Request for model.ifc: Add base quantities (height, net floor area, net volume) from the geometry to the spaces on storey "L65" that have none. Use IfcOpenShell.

First a look at what the model holds.

```python
import ifcopenshell
import ifcopenshell.util.element
import ifcopenshell.util.unit

model = ifcopenshell.open("model.ifc")
print(model.schema)
for unit_type in ("LENGTHUNIT", "AREAUNIT", "VOLUMEUNIT"):
    print(unit_type, ifcopenshell.util.unit.calculate_unit_scale(model, unit_type))
storey = next(s for s in model.by_type("IfcBuildingStorey") if s.Name == "L65")
spaces = [e for e in ifcopenshell.util.element.get_decomposition(storey) if e.is_a("IfcSpace")]
for e in sorted(spaces, key=lambda e: e.id()):
    print(e.id(), e.is_a(), e.Name, list(ifcopenshell.util.element.get_psets(e, qtos_only=True)), sep=" | ")
```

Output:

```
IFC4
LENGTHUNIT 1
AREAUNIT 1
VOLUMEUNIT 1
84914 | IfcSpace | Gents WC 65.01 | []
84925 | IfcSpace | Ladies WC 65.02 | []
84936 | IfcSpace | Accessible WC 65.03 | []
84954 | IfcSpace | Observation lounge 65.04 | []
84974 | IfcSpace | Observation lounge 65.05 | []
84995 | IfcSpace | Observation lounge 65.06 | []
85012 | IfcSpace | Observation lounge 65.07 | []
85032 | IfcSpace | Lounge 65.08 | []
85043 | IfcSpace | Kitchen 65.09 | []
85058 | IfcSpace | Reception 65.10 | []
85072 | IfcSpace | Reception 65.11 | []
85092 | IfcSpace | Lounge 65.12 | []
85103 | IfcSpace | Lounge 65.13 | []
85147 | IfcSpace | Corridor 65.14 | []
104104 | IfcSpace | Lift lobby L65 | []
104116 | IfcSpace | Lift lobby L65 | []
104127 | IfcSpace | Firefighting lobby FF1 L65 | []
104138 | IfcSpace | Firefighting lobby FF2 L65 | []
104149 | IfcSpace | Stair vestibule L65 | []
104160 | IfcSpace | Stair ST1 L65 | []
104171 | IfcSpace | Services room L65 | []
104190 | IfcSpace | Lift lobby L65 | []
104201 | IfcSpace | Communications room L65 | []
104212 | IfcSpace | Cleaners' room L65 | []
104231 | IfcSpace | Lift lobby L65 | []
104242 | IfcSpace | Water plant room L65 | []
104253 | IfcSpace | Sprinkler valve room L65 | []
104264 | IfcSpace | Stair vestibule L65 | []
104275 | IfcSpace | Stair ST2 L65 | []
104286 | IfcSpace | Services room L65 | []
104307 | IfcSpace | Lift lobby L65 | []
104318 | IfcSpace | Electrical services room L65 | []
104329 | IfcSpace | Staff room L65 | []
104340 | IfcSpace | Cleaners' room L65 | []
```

```python
import ifcopenshell
import ifcopenshell.api.pset
import ifcopenshell.geom
import ifcopenshell.util.element
import ifcopenshell.util.shape
import ifcopenshell.util.unit

model = ifcopenshell.open("model.ifc")
unit_scale = ifcopenshell.util.unit.calculate_unit_scale(model)
area_scale = ifcopenshell.util.unit.calculate_unit_scale(model, "AREAUNIT")
volume_scale = ifcopenshell.util.unit.calculate_unit_scale(model, "VOLUMEUNIT")
settings = ifcopenshell.geom.settings()

storey = next(s for s in model.by_type("IfcBuildingStorey") if s.Name == "L65")
spaces = [e for e in ifcopenshell.util.element.get_decomposition(storey) if e.is_a("IfcSpace")]

for e in sorted(spaces, key=lambda e: e.id()):
    if ifcopenshell.util.element.get_psets(e, qtos_only=True, should_inherit=False):
        continue
    # Geometry comes back in metres, in the element's own axes.
    shape = ifcopenshell.geom.create_shape(settings, e)
    values = {
        "Height": ifcopenshell.util.shape.get_z(shape.geometry) / unit_scale,
        "NetFloorArea": ifcopenshell.util.shape.get_footprint_area(shape.geometry) / area_scale,
        "NetVolume": ifcopenshell.util.shape.get_volume(shape.geometry) / volume_scale,
    }
    qto = ifcopenshell.api.pset.add_qto(model, product=e, name="Qto_SpaceBaseQuantities")
    ifcopenshell.api.pset.edit_qto(model, qto=qto, properties=values)
    print(e.id(), {k: round(v, 3) for k, v in values.items()})

model.write("model-out.ifc")
```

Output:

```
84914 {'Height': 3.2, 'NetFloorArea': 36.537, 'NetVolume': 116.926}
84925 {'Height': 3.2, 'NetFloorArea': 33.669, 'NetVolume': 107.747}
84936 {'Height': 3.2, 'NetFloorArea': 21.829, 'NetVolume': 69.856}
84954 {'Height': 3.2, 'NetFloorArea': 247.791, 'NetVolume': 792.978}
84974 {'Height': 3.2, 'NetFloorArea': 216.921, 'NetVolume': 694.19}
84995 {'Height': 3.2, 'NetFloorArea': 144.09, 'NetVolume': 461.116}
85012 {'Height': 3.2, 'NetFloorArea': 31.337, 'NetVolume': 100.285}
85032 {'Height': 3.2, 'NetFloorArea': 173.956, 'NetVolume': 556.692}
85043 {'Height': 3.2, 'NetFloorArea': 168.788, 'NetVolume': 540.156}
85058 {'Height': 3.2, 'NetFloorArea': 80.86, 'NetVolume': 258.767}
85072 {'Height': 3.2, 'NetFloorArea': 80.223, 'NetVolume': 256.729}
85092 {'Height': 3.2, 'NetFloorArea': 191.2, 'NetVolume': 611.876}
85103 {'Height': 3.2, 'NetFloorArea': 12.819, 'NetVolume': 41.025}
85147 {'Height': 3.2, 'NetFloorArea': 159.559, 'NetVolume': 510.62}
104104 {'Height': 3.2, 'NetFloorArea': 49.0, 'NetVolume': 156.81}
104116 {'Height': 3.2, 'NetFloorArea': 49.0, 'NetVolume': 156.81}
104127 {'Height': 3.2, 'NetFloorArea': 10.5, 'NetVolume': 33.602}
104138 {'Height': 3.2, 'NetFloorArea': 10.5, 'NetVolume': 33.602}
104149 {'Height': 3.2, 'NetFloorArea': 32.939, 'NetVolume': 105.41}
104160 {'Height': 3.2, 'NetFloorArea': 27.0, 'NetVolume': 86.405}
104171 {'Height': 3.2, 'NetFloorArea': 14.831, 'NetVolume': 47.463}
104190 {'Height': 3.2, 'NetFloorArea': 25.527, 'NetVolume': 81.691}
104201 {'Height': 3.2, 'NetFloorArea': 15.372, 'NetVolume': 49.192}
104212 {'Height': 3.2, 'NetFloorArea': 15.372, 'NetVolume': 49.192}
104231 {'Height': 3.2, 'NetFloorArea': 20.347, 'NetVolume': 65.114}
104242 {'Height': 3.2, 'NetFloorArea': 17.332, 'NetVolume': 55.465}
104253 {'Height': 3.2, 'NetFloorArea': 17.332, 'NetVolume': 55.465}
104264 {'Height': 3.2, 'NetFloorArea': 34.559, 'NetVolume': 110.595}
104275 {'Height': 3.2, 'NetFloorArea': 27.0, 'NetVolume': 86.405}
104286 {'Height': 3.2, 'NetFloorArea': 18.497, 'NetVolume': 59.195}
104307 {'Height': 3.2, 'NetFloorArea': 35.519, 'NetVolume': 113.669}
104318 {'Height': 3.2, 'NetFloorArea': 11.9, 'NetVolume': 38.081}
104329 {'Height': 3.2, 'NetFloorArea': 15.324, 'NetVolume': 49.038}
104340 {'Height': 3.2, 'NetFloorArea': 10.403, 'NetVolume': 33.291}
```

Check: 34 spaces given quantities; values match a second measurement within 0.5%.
